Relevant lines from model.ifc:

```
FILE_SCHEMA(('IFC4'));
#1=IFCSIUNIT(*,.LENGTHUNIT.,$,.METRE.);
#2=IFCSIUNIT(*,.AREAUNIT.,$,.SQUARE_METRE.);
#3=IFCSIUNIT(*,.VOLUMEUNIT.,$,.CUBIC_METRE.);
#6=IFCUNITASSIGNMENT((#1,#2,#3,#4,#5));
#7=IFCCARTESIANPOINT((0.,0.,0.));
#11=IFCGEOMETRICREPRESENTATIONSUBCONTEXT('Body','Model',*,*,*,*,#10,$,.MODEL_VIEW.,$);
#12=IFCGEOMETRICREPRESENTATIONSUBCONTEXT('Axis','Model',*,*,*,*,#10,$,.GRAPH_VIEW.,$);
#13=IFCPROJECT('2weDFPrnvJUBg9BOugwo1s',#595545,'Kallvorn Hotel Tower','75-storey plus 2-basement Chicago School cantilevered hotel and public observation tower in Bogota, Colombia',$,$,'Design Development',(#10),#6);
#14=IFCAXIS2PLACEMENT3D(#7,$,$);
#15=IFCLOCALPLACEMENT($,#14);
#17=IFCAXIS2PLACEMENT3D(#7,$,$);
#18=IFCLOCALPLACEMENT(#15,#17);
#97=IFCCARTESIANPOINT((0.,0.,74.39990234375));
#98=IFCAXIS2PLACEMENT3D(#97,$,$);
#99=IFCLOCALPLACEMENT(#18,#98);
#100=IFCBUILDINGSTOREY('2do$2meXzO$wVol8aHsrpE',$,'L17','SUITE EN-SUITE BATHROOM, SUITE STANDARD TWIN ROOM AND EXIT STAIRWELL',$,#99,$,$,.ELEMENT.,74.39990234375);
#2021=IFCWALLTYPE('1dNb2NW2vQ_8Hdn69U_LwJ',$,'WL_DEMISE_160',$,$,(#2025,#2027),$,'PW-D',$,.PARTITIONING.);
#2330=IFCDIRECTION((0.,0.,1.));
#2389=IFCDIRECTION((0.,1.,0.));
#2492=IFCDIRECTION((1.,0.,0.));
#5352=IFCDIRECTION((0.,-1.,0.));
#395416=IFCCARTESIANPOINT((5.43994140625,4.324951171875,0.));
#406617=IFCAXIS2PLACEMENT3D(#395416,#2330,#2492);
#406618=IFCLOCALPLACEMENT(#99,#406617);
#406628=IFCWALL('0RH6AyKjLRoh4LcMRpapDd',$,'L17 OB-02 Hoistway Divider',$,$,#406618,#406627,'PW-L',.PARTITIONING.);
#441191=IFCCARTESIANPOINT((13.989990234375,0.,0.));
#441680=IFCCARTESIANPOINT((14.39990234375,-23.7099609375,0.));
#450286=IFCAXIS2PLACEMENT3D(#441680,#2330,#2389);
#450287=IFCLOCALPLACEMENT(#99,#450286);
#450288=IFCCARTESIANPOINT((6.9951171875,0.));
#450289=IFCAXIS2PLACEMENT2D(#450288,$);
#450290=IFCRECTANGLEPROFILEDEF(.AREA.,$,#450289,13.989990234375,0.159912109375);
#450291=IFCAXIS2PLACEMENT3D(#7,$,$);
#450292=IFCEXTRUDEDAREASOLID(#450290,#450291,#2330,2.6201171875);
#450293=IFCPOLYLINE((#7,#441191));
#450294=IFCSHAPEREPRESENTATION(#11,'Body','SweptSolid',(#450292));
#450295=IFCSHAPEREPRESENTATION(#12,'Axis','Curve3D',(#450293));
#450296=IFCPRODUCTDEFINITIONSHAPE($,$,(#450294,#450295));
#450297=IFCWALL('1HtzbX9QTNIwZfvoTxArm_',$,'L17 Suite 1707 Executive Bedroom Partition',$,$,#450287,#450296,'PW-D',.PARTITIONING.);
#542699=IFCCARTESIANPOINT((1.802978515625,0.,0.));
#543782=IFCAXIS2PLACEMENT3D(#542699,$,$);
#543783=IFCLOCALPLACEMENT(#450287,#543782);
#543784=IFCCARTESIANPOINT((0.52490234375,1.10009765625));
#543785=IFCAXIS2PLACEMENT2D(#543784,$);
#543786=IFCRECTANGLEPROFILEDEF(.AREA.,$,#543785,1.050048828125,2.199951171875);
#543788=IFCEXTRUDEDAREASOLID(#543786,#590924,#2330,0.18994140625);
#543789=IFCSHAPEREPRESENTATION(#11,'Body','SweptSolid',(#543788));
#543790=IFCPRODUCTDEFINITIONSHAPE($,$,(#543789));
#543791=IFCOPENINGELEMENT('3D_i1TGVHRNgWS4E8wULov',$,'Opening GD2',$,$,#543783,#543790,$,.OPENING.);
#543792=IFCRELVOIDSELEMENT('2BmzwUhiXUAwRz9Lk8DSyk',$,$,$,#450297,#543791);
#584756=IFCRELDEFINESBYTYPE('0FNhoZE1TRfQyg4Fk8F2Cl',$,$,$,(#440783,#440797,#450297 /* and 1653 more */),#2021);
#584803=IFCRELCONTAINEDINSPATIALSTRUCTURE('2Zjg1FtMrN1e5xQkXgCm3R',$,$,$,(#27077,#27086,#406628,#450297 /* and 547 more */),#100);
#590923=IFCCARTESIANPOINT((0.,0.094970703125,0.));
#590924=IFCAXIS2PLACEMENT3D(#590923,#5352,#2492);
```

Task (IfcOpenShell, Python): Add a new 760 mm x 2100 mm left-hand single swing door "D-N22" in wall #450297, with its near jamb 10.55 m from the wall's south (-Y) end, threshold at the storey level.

```python
import numpy as np
import ifcopenshell
import ifcopenshell.api.feature
import ifcopenshell.api.geometry
import ifcopenshell.api.root
import ifcopenshell.api.spatial
import ifcopenshell.geom
import ifcopenshell.util.element
import ifcopenshell.util.placement
import ifcopenshell.util.representation
import ifcopenshell.util.shape
import ifcopenshell.util.unit

model = ifcopenshell.open("model.ifc")
unit_scale = ifcopenshell.util.unit.calculate_unit_scale(model)
settings = ifcopenshell.geom.settings()


def volume(element):
    """Net volume in cubic metres, openings subtracted."""
    shape = ifcopenshell.geom.create_shape(settings, element)
    return ifcopenshell.util.shape.get_volume(shape.geometry)


wall = model.by_id(450297)
storey = ifcopenshell.util.element.get_container(wall, ifc_class="IfcBuildingStorey")
context = ifcopenshell.util.representation.get_context(model, "Model", "Body", "MODEL_VIEW")
before = volume(wall)

width, height, from_end, sill = 0.76, 2.1, 10.55, 0.0  # metres

# The wall runs along its own X axis, and the end named is its -X end.
wall_shape = ifcopenshell.geom.create_shape(settings, wall)
x, y, z = ifcopenshell.util.shape.get_vertices(wall_shape.geometry).T
start = x.min() + from_end
face, thickness = float(y.min()), float(y.max() - y.min())
wall_matrix = ifcopenshell.util.placement.get_local_placement(wall.ObjectPlacement)
level = ifcopenshell.util.placement.get_local_placement(storey.ObjectPlacement)[2, 3]


def in_wall(x, y):
    """Placement at x, y metres in the wall's axes, at sill height."""
    matrix = wall_matrix.copy()
    matrix[:, 3] = wall_matrix @ np.array([x / unit_scale, y / unit_scale, 0.0, 1.0])
    matrix[2, 3] = level + sill / unit_scale
    return matrix


# Opening: a box that overshoots both wall faces by 50 mm.
opening = ifcopenshell.api.root.create_entity(model, ifc_class="IfcOpeningElement", predefined_type="OPENING")
box = ifcopenshell.api.geometry.add_wall_representation(
    model, context=context, length=width, height=height, thickness=thickness + 0.1
)
ifcopenshell.api.geometry.assign_representation(model, product=opening, representation=box)
ifcopenshell.api.geometry.edit_object_placement(model, product=opening, matrix=in_wall(start, face - 0.05), is_si=False)
ifcopenshell.api.feature.add_feature(model, feature=opening, element=wall)

door = ifcopenshell.api.root.create_entity(model, ifc_class="IfcDoor", name="D-N22", predefined_type="DOOR")
door.OverallWidth, door.OverallHeight = width / unit_scale, height / unit_scale
door.OperationType = "SINGLE_SWING_LEFT"
body = ifcopenshell.api.geometry.add_door_representation(
    model,
    context=context,
    overall_width=door.OverallWidth,
    overall_height=door.OverallHeight,
    operation_type="SINGLE_SWING_LEFT",
    lining_properties={"LiningDepth": thickness / unit_scale, "ThresholdDepth": thickness / unit_scale},
)
ifcopenshell.api.geometry.assign_representation(model, product=door, representation=body)
ifcopenshell.api.spatial.assign_container(model, products=[door], relating_structure=storey)
ifcopenshell.api.feature.add_filling(model, opening=opening, element=door)

# The lining spans the wall, so the door starts at the wall face.
ifcopenshell.api.geometry.edit_object_placement(model, product=door, matrix=in_wall(start, face), is_si=False)

after = volume(wall)

print(f"wall volume {before:.3f} -> {after:.3f} m3")

model.write("model_updated.ifc")
```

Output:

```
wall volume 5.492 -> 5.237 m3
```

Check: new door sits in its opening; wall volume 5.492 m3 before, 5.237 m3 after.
